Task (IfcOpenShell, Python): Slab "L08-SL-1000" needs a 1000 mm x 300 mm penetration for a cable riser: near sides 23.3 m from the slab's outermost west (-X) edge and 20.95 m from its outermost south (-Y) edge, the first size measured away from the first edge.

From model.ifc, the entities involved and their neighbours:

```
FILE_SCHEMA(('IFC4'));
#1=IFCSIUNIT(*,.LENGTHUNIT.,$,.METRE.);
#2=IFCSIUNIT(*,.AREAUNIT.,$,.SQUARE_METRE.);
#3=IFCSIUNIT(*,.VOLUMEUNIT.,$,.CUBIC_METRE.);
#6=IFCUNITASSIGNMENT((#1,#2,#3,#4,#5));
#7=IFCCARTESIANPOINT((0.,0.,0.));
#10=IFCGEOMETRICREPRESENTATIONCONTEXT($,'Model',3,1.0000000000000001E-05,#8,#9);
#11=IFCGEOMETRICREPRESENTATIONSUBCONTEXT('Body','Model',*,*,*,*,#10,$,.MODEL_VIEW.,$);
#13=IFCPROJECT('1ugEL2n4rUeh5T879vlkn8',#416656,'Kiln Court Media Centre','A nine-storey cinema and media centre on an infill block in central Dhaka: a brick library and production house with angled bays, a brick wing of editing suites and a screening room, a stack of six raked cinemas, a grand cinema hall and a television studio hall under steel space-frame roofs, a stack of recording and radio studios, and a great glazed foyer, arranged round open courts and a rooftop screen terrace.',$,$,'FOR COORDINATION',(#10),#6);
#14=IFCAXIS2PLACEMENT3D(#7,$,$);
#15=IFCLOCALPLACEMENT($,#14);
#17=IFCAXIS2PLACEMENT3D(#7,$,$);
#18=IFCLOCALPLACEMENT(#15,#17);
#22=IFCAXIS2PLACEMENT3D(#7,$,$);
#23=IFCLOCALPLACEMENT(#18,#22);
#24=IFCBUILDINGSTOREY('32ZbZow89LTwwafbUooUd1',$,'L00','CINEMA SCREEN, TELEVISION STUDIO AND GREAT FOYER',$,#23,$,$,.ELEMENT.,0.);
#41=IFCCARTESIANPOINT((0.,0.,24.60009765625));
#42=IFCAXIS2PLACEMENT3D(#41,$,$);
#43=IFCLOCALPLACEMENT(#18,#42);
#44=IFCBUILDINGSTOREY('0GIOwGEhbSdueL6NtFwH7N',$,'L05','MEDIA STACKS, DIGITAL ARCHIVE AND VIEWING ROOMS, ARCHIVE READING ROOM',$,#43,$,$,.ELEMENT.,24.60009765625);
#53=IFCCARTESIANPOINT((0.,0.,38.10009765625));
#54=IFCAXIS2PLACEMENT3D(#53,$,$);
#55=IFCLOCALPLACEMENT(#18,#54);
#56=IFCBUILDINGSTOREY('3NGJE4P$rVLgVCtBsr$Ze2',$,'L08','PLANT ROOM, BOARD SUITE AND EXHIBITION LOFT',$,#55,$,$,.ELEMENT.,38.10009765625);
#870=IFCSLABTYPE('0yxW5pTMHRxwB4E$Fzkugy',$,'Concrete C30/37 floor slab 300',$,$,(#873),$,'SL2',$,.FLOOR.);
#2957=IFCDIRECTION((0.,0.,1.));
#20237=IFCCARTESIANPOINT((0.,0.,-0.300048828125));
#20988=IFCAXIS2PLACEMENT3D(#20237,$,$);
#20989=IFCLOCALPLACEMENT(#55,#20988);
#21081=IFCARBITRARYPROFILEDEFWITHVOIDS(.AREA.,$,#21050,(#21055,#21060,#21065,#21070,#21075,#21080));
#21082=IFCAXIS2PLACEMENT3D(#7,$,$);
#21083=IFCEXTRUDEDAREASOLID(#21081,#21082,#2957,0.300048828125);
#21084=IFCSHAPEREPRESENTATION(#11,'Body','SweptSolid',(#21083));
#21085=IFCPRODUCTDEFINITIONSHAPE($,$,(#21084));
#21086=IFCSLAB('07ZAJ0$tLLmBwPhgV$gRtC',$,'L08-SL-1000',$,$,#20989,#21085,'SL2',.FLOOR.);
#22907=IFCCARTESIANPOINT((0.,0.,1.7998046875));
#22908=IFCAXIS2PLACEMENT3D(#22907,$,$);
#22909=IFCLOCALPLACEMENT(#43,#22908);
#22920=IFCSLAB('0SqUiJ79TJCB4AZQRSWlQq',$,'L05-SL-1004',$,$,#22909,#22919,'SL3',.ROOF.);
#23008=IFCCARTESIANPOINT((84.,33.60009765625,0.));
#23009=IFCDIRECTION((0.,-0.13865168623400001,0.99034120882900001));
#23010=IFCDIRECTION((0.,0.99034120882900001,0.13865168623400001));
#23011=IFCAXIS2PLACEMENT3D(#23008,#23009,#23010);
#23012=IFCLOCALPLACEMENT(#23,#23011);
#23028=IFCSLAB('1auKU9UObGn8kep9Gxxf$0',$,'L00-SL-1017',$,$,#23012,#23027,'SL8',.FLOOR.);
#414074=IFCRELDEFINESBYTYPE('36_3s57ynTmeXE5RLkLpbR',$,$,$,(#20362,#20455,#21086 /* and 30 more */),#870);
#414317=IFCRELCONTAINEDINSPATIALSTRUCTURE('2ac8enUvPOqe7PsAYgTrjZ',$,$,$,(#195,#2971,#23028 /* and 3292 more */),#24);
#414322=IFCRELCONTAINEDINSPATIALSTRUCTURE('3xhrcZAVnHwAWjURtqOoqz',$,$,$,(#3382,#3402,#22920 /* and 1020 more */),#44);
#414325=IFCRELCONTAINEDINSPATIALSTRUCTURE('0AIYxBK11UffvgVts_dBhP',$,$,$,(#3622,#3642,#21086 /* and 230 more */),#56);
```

```python
import numpy as np
import ifcopenshell
import ifcopenshell.api.feature
import ifcopenshell.api.geometry
import ifcopenshell.api.root
import ifcopenshell.geom
import ifcopenshell.util.placement
import ifcopenshell.util.representation
import ifcopenshell.util.shape
import ifcopenshell.util.unit

model = ifcopenshell.open("model.ifc")
unit_scale = ifcopenshell.util.unit.calculate_unit_scale(model)
settings = ifcopenshell.geom.settings()


def volume(element):
    """Net volume in cubic metres, openings subtracted."""
    shape = ifcopenshell.geom.create_shape(settings, element)
    return ifcopenshell.util.shape.get_volume(shape.geometry)


slab = model.by_guid("07ZAJ0$tLLmBwPhgV$gRtC")
before = volume(slab)

# Extent in the slab's own axes, in metres. The edges named are its -X and -Y sides.
slab_shape = ifcopenshell.geom.create_shape(settings, slab)
vertices = ifcopenshell.util.shape.get_vertices(slab_shape.geometry)
x_min, y_min, bottom = vertices.min(axis=0)
top = vertices[:, 2].max()

opening = ifcopenshell.api.root.create_entity(model, ifc_class="IfcOpeningElement", name="Cable riser opening", predefined_type="OPENING")
context = ifcopenshell.util.representation.get_context(model, "Model", "Body", "MODEL_VIEW")
width, depth = 1, 0.3
outline = [(0.0, 0.0), (width, 0.0), (width, depth), (0.0, depth), (0.0, 0.0)]
# Overshoot both faces by 50 mm so the cut is clean.
shape = ifcopenshell.api.geometry.add_slab_representation(
    model, context=context, depth=top - bottom + 0.1, polyline=outline
)
ifcopenshell.api.geometry.assign_representation(model, product=opening, representation=shape)

matrix = ifcopenshell.util.placement.get_local_placement(slab.ObjectPlacement)
matrix[:, 3] = matrix @ np.append(np.array([x_min + 23.3, y_min + 20.95, bottom - 0.05]) / unit_scale, 1.0)
ifcopenshell.api.geometry.edit_object_placement(model, product=opening, matrix=matrix, is_si=False)
ifcopenshell.api.feature.add_feature(model, feature=opening, element=slab)

after = volume(slab)

print(f"slab volume {before:.3f} -> {after:.3f} m3")

model.write("model_v2.ifc")
```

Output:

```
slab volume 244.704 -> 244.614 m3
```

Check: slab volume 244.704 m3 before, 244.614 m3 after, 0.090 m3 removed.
